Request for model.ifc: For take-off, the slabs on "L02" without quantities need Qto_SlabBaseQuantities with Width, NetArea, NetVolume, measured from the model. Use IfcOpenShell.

First a look at what the model holds.

```python
import ifcopenshell
import ifcopenshell.util.element
import ifcopenshell.util.unit

model = ifcopenshell.open("model.ifc")
print(model.schema)
for unit_type in ("LENGTHUNIT", "AREAUNIT", "VOLUMEUNIT"):
    print(unit_type, ifcopenshell.util.unit.calculate_unit_scale(model, unit_type))
storey = next(s for s in model.by_type("IfcBuildingStorey") if s.Name == "L02")
slabs = [e for e in ifcopenshell.util.element.get_decomposition(storey) if e.is_a("IfcSlab")]
for e in sorted(slabs, key=lambda e: e.id()):
    print(e.id(), e.is_a(), e.Name, list(ifcopenshell.util.element.get_psets(e, qtos_only=True)), sep=" | ")
```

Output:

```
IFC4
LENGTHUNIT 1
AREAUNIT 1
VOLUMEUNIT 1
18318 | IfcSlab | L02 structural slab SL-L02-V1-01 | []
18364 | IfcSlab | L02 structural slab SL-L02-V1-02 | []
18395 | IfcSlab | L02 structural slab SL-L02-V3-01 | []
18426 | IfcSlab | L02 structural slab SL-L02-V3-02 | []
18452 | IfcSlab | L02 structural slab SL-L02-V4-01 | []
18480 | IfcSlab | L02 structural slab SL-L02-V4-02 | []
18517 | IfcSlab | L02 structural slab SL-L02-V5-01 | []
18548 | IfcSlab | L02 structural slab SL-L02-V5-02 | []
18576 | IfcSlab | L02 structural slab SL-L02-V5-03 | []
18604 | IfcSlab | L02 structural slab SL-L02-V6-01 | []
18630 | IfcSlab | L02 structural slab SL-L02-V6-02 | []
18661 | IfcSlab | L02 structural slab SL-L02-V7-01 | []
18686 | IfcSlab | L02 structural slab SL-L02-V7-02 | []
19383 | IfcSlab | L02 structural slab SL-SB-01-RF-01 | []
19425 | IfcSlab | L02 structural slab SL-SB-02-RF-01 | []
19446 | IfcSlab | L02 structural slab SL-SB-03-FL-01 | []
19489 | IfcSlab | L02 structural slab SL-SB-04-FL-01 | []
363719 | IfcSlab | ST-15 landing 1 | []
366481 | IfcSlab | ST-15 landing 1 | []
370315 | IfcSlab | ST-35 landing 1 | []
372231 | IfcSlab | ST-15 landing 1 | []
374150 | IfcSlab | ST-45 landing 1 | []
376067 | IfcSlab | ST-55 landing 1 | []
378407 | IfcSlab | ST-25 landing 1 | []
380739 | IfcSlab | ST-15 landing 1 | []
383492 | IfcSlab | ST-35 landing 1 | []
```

```python
import ifcopenshell
import ifcopenshell.api.pset
import ifcopenshell.geom
import ifcopenshell.util.element
import ifcopenshell.util.shape
import ifcopenshell.util.unit

model = ifcopenshell.open("model.ifc")
unit_scale = ifcopenshell.util.unit.calculate_unit_scale(model)
area_scale = ifcopenshell.util.unit.calculate_unit_scale(model, "AREAUNIT")
volume_scale = ifcopenshell.util.unit.calculate_unit_scale(model, "VOLUMEUNIT")
settings = ifcopenshell.geom.settings()

storey = next(s for s in model.by_type("IfcBuildingStorey") if s.Name == "L02")
slabs = [e for e in ifcopenshell.util.element.get_decomposition(storey) if e.is_a("IfcSlab")]

for e in sorted(slabs, key=lambda e: e.id()):
    if ifcopenshell.util.element.get_psets(e, qtos_only=True, should_inherit=False):
        continue
    # Geometry comes back in metres, in the element's own axes.
    shape = ifcopenshell.geom.create_shape(settings, e)
    values = {
        "Width": ifcopenshell.util.shape.get_z(shape.geometry) / unit_scale,
        "NetArea": ifcopenshell.util.shape.get_footprint_area(shape.geometry) / area_scale,
        "NetVolume": ifcopenshell.util.shape.get_volume(shape.geometry) / volume_scale,
    }
    qto = ifcopenshell.api.pset.add_qto(model, product=e, name="Qto_SlabBaseQuantities")
    ifcopenshell.api.pset.edit_qto(model, qto=qto, properties=values)
    print(e.id(), {k: round(v, 3) for k, v in values.items()})

model.write("model_edited.ifc")
```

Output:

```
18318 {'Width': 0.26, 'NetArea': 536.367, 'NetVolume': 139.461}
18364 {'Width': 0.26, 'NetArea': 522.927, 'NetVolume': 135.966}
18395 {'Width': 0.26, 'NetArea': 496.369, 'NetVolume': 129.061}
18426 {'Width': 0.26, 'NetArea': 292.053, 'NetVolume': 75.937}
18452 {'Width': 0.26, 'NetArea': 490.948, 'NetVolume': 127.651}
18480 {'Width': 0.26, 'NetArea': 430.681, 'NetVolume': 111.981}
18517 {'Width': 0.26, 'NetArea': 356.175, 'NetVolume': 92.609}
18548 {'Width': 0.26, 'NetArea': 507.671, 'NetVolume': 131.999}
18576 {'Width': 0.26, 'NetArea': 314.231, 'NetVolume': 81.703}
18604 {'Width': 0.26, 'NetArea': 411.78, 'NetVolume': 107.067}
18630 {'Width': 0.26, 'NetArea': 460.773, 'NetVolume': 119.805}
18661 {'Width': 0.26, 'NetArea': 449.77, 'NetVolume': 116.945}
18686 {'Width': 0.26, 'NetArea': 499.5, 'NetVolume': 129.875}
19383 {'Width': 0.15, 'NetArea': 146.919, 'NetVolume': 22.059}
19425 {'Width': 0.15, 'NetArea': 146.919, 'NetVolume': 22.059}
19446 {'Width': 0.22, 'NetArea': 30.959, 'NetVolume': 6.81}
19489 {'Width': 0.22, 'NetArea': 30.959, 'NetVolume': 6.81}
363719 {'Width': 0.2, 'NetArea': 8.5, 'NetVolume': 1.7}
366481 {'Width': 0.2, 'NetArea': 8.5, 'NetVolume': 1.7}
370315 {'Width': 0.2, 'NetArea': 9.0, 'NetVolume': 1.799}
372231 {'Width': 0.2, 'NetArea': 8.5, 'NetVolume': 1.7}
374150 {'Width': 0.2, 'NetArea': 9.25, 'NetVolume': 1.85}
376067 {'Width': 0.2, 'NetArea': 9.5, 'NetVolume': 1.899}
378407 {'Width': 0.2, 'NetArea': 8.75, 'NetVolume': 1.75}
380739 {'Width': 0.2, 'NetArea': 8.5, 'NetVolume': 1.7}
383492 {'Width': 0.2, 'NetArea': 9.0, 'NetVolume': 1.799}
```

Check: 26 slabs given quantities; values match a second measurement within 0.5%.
